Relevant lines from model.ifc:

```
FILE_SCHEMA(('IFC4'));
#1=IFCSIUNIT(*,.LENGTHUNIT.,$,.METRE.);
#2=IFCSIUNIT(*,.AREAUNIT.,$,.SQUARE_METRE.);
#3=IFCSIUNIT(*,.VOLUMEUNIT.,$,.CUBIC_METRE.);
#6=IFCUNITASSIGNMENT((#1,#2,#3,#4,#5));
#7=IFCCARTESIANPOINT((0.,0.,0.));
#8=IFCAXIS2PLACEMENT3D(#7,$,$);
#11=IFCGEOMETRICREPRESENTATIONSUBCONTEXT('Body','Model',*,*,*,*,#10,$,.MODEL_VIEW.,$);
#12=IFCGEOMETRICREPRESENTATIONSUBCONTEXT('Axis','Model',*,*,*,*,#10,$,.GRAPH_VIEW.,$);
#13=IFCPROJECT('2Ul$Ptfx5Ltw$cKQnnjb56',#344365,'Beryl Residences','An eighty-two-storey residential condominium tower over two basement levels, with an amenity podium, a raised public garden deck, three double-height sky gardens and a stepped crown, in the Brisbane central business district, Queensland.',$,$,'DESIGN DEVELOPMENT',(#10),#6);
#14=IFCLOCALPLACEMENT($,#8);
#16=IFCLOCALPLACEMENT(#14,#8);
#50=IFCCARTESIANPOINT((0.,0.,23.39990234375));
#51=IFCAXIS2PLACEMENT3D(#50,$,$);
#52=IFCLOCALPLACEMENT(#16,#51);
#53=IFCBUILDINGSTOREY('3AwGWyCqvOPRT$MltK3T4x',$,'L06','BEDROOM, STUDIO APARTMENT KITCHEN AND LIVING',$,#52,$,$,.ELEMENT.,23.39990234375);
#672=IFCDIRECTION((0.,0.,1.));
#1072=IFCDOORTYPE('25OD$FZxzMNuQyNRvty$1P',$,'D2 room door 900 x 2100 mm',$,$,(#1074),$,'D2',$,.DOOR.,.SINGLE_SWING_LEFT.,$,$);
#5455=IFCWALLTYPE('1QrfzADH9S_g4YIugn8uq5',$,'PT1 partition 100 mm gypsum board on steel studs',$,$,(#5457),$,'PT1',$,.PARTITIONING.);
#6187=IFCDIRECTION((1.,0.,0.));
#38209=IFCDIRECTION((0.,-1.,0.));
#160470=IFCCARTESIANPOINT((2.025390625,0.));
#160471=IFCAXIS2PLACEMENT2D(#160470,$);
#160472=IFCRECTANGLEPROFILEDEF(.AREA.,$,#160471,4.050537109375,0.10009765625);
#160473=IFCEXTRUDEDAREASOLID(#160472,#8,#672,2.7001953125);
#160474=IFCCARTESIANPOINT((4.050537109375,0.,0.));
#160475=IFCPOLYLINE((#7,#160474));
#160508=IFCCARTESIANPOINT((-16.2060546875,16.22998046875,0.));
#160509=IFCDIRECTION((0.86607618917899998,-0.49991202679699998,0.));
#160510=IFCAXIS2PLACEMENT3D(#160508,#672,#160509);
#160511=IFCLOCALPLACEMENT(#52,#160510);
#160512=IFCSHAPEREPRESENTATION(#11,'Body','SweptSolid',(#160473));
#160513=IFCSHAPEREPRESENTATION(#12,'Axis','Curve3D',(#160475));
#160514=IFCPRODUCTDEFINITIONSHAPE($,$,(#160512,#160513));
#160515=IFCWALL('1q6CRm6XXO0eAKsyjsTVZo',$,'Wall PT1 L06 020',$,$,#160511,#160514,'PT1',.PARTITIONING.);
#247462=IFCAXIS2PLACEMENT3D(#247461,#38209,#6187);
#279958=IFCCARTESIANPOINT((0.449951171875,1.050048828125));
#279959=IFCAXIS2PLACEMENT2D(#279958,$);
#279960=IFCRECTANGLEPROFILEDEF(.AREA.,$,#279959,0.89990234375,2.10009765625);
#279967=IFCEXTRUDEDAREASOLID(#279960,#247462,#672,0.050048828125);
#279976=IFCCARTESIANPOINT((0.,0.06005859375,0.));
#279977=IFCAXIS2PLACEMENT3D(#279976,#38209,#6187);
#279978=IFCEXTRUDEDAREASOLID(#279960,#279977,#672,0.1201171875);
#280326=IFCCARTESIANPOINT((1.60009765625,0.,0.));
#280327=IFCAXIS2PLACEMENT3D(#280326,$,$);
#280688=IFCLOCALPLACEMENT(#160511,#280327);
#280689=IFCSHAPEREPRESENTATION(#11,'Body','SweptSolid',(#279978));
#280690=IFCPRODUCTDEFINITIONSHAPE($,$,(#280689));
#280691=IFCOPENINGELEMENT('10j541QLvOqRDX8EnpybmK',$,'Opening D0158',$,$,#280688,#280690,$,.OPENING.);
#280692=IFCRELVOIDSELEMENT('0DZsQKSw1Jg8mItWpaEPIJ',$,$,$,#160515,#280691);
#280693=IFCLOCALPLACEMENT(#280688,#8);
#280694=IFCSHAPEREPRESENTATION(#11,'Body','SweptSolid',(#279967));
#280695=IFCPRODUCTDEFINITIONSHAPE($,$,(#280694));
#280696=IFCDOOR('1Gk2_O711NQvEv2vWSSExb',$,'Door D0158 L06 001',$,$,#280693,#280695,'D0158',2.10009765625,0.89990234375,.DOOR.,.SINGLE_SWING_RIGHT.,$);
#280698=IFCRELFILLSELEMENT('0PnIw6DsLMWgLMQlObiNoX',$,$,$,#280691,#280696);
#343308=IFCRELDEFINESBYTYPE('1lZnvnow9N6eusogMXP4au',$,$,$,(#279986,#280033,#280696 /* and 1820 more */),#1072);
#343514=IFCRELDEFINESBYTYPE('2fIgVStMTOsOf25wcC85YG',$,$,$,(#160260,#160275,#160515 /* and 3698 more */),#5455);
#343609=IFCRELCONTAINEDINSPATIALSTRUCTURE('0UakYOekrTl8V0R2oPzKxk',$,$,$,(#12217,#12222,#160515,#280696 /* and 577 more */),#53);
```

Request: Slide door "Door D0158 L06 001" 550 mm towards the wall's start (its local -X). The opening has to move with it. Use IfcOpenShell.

```python
import ifcopenshell
import ifcopenshell.api.geometry
import ifcopenshell.util.placement

model = ifcopenshell.open("model.ifc")

door = model.by_id(280696)
opening = door.FillsVoids[0].RelatingOpeningElement
wall = opening.VoidsElements[0].RelatingBuildingElement

wall_matrix = ifcopenshell.util.placement.get_local_placement(wall.ObjectPlacement)
shift = wall_matrix[:3, 0] * -0.55
before = ifcopenshell.util.placement.get_local_placement(door.ObjectPlacement)[:3, 3].copy()

# The door is placed relative to its opening, so it follows when the opening moves.
matrix = ifcopenshell.util.placement.get_local_placement(opening.ObjectPlacement)
matrix[:3, 3] += shift
ifcopenshell.api.geometry.edit_object_placement(
    model, product=opening, matrix=matrix, is_si=False, should_transform_children=True
)

after = ifcopenshell.util.placement.get_local_placement(door.ObjectPlacement)[:3, 3]
print("door moved by", (after - before).round(3) + 0.0)

model.write("model-out.ifc")
```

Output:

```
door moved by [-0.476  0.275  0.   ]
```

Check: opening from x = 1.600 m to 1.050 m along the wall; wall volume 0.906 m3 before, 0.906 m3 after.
